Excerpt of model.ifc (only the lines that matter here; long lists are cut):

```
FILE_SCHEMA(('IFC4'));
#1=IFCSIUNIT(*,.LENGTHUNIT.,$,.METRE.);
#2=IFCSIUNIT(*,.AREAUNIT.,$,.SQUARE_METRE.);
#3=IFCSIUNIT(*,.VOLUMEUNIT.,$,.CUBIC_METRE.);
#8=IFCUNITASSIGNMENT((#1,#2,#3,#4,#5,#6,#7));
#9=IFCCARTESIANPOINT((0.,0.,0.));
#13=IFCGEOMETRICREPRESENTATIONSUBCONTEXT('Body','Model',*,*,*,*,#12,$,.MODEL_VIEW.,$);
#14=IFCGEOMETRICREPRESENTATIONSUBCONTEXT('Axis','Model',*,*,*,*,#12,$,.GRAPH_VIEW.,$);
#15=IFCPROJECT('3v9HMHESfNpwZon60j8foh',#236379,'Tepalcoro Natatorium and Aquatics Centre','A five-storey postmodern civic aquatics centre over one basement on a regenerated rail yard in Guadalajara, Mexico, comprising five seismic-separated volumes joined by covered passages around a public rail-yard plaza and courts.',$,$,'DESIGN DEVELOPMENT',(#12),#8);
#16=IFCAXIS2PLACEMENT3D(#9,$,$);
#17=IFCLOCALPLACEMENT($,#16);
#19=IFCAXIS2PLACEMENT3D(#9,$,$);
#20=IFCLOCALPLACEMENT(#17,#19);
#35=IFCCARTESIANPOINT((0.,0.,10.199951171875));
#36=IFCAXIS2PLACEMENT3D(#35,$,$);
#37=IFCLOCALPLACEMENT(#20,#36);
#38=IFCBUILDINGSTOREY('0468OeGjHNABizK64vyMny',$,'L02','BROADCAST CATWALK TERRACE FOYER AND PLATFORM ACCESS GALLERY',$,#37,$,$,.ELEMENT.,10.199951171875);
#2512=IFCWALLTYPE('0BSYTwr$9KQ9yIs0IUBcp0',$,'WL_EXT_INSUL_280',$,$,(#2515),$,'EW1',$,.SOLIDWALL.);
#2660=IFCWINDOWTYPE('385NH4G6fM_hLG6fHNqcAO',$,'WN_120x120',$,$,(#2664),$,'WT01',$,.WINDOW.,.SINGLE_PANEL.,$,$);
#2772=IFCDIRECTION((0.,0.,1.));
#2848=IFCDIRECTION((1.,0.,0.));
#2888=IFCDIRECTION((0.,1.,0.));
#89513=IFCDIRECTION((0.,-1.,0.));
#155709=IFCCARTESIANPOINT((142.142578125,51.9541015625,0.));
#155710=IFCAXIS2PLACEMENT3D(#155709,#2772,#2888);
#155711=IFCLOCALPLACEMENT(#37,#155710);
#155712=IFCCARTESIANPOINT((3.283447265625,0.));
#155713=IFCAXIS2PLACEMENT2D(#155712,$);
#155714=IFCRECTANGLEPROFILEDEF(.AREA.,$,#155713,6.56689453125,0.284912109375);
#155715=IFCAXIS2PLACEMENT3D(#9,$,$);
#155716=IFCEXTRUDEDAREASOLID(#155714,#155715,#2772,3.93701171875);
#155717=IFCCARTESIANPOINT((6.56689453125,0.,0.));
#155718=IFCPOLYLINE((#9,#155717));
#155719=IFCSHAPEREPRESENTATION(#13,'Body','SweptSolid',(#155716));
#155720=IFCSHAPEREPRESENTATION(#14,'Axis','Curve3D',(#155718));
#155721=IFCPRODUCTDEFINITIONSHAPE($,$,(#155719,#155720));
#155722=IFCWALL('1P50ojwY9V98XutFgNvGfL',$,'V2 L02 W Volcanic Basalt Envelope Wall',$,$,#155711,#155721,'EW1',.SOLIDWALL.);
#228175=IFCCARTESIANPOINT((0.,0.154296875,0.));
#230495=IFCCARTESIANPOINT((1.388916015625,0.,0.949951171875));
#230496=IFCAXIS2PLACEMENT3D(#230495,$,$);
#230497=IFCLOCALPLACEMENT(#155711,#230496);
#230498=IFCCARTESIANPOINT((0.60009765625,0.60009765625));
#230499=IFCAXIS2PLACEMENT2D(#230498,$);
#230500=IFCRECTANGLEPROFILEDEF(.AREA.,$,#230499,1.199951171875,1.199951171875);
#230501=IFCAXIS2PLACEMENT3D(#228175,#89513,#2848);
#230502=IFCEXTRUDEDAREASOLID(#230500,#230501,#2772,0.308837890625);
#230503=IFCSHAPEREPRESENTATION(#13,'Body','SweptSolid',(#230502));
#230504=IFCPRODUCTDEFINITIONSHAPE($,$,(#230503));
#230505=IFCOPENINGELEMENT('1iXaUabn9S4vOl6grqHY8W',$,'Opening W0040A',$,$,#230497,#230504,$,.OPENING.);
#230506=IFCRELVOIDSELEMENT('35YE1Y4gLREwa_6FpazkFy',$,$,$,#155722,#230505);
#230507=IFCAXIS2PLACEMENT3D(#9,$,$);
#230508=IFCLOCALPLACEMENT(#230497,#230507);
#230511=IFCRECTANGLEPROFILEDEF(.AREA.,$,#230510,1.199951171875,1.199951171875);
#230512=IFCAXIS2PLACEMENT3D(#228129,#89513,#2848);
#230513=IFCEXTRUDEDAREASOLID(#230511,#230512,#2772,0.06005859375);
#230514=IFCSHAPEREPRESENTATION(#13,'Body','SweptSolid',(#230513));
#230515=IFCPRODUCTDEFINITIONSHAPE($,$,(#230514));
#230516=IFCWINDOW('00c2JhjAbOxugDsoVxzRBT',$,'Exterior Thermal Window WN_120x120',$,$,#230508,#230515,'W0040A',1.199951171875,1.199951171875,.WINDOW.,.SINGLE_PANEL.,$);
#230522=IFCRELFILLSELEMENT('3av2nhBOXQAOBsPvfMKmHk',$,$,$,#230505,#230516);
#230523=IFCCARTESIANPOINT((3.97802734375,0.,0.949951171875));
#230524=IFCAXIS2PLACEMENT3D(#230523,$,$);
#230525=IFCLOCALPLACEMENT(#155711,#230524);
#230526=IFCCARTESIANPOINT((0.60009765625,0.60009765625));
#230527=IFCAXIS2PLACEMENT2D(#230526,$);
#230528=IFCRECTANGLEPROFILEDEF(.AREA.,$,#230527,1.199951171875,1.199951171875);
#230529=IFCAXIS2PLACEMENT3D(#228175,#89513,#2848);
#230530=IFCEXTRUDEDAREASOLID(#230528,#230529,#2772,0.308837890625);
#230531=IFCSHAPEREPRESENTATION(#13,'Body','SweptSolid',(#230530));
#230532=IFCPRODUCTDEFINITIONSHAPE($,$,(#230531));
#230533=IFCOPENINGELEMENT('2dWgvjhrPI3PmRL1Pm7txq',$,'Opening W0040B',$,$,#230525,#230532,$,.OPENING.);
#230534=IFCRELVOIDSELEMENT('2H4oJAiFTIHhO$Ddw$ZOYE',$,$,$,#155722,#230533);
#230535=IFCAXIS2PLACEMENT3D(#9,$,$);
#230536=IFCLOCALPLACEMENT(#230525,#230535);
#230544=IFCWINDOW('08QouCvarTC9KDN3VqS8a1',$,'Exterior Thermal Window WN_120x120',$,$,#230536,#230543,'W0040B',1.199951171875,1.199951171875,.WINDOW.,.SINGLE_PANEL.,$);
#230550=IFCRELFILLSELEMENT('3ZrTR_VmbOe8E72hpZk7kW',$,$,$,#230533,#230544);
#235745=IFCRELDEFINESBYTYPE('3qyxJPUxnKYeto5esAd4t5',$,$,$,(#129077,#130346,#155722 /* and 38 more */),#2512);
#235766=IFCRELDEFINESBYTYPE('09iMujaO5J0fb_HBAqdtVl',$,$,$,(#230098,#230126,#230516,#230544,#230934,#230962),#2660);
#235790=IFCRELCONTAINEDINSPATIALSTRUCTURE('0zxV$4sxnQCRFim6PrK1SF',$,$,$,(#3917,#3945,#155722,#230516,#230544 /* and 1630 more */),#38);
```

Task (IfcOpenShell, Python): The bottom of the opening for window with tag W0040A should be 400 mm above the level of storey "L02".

```python
import numpy as np
import ifcopenshell
import ifcopenshell.api.geometry
import ifcopenshell.geom
import ifcopenshell.util.element
import ifcopenshell.util.placement
import ifcopenshell.util.shape
import ifcopenshell.util.unit

model = ifcopenshell.open("model.ifc")
unit_scale = ifcopenshell.util.unit.calculate_unit_scale(model)

window = model.by_guid("00c2JhjAbOxugDsoVxzRBT")
opening = window.FillsVoids[0].RelatingOpeningElement
storey = ifcopenshell.util.element.get_container(window, ifc_class="IfcBuildingStorey")
level = ifcopenshell.util.placement.get_local_placement(storey.ObjectPlacement)[2, 3]

# The opening's origin need not be at the sill, so measure its lowest point.
shape = ifcopenshell.geom.create_shape(ifcopenshell.geom.settings(), opening)
bottom = ifcopenshell.util.shape.get_shape_bottom_elevation(shape, shape.geometry) / unit_scale
dz = level + 0.4 - bottom

shift = np.array([0.0, 0.0, dz])
# The window is placed relative to its opening, so it follows when the opening moves.
matrix = ifcopenshell.util.placement.get_local_placement(opening.ObjectPlacement)
matrix[:3, 3] += shift
ifcopenshell.api.geometry.edit_object_placement(
    model, product=opening, matrix=matrix, is_si=False, should_transform_children=True
)

print(f"moved by {dz * unit_scale:+.3f} m")

model.write("model_v2.ifc")
```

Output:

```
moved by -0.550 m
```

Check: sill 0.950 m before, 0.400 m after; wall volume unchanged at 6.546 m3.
